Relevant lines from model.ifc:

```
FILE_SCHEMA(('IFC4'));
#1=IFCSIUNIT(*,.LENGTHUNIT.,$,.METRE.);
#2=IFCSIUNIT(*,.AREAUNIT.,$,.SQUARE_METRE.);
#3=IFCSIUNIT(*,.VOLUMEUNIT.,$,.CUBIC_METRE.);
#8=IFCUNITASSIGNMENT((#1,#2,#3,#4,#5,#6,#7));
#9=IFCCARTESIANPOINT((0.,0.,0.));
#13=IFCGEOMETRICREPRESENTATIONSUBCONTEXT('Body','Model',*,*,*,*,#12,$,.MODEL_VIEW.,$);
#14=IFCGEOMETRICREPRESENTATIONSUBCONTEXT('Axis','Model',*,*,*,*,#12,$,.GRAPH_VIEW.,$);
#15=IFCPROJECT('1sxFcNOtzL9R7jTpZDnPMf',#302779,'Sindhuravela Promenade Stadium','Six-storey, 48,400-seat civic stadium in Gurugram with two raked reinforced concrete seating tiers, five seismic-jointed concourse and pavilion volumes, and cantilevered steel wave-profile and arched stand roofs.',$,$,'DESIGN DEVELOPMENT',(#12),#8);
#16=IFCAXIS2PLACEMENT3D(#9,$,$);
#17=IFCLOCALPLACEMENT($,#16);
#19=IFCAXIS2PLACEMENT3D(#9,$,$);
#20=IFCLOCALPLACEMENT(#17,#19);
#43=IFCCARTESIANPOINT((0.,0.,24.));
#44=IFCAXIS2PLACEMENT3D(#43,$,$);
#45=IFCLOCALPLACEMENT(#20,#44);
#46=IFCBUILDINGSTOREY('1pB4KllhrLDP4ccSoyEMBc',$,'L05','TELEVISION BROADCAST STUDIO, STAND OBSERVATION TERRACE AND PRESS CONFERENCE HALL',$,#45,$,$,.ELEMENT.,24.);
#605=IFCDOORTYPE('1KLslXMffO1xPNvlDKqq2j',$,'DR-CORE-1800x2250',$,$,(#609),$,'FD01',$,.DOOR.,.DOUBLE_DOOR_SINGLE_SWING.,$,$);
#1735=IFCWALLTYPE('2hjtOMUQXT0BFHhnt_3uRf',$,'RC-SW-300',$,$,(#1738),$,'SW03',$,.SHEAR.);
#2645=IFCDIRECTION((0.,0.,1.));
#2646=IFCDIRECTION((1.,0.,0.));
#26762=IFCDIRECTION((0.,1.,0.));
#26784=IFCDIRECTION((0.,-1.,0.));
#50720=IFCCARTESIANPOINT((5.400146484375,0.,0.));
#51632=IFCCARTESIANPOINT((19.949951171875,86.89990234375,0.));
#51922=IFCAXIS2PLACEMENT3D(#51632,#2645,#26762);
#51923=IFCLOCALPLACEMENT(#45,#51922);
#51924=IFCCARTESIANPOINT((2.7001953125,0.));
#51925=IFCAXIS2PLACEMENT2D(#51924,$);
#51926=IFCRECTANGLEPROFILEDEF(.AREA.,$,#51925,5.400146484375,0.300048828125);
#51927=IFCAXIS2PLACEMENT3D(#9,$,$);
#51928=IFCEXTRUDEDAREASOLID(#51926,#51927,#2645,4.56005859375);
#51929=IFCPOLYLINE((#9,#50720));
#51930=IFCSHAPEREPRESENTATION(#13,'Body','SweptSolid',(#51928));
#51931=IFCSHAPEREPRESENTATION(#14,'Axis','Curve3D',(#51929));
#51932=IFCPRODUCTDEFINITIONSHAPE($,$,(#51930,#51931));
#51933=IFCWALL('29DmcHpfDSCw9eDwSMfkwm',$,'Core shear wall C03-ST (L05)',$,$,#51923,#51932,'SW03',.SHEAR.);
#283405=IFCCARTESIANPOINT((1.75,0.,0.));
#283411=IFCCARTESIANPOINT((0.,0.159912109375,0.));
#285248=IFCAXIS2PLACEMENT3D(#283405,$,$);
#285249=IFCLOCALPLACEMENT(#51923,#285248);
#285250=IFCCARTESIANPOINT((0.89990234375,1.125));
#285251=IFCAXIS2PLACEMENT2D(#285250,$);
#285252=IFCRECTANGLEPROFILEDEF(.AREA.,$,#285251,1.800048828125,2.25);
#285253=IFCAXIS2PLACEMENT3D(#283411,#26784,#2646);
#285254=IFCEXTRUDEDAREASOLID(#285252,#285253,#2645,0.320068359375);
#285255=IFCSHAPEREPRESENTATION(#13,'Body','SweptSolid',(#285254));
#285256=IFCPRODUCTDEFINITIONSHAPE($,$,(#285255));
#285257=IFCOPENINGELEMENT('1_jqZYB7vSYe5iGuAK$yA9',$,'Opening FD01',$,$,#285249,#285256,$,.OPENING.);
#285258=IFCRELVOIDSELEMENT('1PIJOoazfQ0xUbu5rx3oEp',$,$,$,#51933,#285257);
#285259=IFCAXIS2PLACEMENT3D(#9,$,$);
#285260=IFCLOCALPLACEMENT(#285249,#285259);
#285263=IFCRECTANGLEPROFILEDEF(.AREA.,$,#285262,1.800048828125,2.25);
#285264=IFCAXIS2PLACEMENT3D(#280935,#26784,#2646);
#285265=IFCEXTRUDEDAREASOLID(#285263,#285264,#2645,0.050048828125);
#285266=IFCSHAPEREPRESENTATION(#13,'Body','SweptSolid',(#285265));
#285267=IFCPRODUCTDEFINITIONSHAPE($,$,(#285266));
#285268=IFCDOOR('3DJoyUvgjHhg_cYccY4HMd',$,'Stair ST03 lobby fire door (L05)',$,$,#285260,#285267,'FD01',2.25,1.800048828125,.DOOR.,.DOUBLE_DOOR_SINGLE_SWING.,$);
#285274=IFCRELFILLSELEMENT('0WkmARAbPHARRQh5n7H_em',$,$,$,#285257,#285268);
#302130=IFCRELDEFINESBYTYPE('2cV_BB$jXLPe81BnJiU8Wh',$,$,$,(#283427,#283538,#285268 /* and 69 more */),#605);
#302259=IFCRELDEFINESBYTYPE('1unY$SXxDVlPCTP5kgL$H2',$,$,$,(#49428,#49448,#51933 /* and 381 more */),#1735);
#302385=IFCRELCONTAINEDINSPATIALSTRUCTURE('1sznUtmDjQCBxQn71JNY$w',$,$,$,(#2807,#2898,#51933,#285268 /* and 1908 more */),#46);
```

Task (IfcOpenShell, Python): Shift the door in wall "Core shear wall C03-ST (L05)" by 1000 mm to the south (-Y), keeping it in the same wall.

```python
import ifcopenshell
import ifcopenshell.api.geometry
import ifcopenshell.util.placement
import ifcopenshell.util.unit

model = ifcopenshell.open("model.ifc")
unit_scale = ifcopenshell.util.unit.calculate_unit_scale(model)

door = model.by_id(285268)
opening = door.FillsVoids[0].RelatingOpeningElement
wall = opening.VoidsElements[0].RelatingBuildingElement

wall_matrix = ifcopenshell.util.placement.get_local_placement(wall.ObjectPlacement)
shift = wall_matrix[:3, 0] * -1 / unit_scale
before = ifcopenshell.util.placement.get_local_placement(door.ObjectPlacement)[:3, 3].copy()

# The door is placed relative to its opening, so it follows when the opening moves.
matrix = ifcopenshell.util.placement.get_local_placement(opening.ObjectPlacement)
matrix[:3, 3] += shift
ifcopenshell.api.geometry.edit_object_placement(
    model, product=opening, matrix=matrix, is_si=False, should_transform_children=True
)

after = ifcopenshell.util.placement.get_local_placement(door.ObjectPlacement)[:3, 3]
print("door moved by", (after - before).round(3) + 0.0)

model.write("model_edited.ifc")
```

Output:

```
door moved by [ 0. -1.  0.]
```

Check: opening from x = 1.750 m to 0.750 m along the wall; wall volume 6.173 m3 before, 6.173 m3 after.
